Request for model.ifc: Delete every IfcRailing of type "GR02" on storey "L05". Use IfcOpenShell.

First a look at what the model holds.

```python
import ifcopenshell
import ifcopenshell.util.element

model = ifcopenshell.open("model.ifc")
print(model.schema)
storey = next(s for s in model.by_type("IfcBuildingStorey") if s.Name == "L05")
railings = [e for e in ifcopenshell.util.element.get_decomposition(storey) if e.is_a("IfcRailing")]
seen = {}
for e in railings:
    element_type = ifcopenshell.util.element.get_type(e)
    name = element_type.Name if element_type not in (None, e) else None
    seen[name] = seen.get(name, 0) + 1
for name, count in sorted(seen.items(), key=str):
    print(count, "x", name)
```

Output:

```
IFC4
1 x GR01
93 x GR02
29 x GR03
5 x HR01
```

```python
import ifcopenshell
import ifcopenshell.api.root
import ifcopenshell.util.element

model = ifcopenshell.open("model.ifc")

storey = next(s for s in model.by_type("IfcBuildingStorey") if s.Name == "L05")
railings = [e for e in ifcopenshell.util.element.get_decomposition(storey) if e.is_a("IfcRailing")]
targets = [e for e in railings if (t := ifcopenshell.util.element.get_type(e)) not in (None, e) and t.Name == "GR02"]

for e in targets:
    ifcopenshell.api.root.remove_product(model, product=e)
print(len(targets), "removed")

model.write("model_edited.ifc")
```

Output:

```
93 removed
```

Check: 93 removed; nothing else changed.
